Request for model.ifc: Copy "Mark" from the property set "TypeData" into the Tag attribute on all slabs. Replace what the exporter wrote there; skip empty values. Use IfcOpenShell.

First a look at what the model holds.

```python
import ifcopenshell
import ifcopenshell.util.element

model = ifcopenshell.open("model.ifc")
print(model.schema)
slabs = model.by_type("IfcSlab")
print(len(slabs), "slabs")
for e in slabs[:8]:
    source = ifcopenshell.util.element.get_pset(e, "TypeData", "Mark")
    target = e.Tag
    print(e.id(), repr(source), repr(target), sep=" | ")
```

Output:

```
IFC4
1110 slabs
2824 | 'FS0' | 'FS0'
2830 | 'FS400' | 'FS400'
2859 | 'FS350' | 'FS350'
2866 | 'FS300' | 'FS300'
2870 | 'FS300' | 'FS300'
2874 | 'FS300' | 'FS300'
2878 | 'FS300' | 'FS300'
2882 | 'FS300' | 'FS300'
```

```python
import ifcopenshell
import ifcopenshell.util.element

model = ifcopenshell.open("model.ifc")

count = 0
for e in model.by_type("IfcSlab"):
    value = ifcopenshell.util.element.get_pset(e, "TypeData", "Mark")
    current = e.Tag
    if not value or not value.strip() or current == value:
        continue
    e.Tag = value
    count += 1

print(count, "slabs updated")

model.write("model_updated.ifc")
```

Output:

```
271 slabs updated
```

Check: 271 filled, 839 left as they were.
